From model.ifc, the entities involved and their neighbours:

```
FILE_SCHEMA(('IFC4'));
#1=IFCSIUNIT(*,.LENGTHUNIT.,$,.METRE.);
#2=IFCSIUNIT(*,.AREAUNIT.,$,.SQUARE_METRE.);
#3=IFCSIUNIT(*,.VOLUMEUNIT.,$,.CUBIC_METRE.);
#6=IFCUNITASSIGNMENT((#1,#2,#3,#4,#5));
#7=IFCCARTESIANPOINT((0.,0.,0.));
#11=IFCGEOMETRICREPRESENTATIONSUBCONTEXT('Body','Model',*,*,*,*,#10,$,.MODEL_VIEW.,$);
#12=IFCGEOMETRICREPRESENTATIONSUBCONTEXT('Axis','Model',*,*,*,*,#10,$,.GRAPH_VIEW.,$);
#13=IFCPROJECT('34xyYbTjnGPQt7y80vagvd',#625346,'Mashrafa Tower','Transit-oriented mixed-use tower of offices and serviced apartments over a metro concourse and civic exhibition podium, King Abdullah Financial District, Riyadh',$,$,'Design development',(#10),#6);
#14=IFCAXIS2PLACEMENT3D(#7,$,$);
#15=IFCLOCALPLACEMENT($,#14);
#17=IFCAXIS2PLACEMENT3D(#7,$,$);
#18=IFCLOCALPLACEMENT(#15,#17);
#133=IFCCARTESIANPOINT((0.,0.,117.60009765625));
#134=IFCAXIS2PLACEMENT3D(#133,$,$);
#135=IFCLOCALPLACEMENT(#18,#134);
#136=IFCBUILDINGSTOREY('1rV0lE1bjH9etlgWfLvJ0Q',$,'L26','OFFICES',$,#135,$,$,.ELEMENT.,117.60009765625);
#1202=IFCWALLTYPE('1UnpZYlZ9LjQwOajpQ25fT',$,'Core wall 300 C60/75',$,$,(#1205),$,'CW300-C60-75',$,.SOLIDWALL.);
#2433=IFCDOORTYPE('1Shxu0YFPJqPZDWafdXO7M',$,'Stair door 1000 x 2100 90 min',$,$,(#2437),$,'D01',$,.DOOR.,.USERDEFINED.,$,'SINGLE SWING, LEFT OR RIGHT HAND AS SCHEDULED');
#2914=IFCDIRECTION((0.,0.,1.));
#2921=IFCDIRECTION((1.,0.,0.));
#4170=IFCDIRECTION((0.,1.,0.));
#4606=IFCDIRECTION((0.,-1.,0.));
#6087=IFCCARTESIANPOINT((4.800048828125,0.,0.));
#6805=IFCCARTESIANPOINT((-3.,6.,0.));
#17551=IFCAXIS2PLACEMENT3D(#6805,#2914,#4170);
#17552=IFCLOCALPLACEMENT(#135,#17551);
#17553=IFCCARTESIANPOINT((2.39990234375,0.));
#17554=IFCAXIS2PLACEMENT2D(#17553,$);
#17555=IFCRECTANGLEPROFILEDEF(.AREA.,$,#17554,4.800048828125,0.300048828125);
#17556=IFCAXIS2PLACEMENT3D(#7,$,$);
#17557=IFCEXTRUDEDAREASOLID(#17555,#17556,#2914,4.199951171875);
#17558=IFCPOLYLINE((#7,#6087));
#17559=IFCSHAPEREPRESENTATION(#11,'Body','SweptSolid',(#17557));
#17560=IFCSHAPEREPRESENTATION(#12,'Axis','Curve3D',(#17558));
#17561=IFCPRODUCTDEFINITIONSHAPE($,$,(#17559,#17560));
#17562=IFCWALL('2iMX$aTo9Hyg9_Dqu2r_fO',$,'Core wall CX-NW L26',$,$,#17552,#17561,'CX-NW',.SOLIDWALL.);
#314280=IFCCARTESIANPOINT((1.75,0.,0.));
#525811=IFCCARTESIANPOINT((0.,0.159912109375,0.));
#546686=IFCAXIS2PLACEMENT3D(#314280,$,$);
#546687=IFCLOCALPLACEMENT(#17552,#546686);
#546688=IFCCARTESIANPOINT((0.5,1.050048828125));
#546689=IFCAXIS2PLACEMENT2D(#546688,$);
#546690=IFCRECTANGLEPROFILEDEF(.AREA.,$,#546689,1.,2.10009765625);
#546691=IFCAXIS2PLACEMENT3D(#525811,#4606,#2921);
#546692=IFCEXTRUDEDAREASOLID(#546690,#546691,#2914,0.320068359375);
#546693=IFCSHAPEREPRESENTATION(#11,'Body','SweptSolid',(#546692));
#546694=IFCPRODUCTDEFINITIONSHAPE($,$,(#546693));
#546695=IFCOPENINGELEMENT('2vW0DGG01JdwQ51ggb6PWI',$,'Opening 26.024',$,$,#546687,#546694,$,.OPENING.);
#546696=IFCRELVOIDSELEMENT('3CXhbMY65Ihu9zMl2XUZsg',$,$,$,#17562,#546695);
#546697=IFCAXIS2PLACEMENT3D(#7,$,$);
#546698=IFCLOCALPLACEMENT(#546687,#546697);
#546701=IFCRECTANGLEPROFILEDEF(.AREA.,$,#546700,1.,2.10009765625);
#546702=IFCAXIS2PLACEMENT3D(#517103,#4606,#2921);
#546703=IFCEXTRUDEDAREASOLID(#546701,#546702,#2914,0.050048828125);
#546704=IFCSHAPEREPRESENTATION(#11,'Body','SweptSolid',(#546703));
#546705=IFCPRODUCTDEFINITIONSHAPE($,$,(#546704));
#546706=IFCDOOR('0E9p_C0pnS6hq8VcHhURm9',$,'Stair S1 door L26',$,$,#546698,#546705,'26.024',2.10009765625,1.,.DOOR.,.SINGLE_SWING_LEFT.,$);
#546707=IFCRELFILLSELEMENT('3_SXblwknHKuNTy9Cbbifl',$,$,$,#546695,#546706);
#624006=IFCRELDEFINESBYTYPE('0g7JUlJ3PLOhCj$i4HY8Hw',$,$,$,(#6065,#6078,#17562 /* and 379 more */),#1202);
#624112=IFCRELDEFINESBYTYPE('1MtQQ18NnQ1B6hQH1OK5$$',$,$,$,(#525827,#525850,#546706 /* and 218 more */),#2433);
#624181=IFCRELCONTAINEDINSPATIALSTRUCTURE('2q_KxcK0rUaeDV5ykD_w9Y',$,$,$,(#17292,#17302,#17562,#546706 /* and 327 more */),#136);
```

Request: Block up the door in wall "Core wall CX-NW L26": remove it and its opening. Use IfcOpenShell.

```python
import ifcopenshell
import ifcopenshell.api.feature
import ifcopenshell.api.root
import ifcopenshell.geom
import ifcopenshell.util.shape

model = ifcopenshell.open("model.ifc")
settings = ifcopenshell.geom.settings()


def volume(element):
    """Net volume in cubic metres, openings subtracted."""
    shape = ifcopenshell.geom.create_shape(settings, element)
    return ifcopenshell.util.shape.get_volume(shape.geometry)


door = model.by_guid("0E9p_C0pnS6hq8VcHhURm9")
opening = door.FillsVoids[0].RelatingOpeningElement
wall = opening.VoidsElements[0].RelatingBuildingElement
before = volume(wall)

ifcopenshell.api.root.remove_product(model, product=door)
ifcopenshell.api.feature.remove_feature(model, feature=opening)

after = volume(wall)

print(f"wall volume {before:.3f} -> {after:.3f} m3")

model.write("model_updated.ifc")
```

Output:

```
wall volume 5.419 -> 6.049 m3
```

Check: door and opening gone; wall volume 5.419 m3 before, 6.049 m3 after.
